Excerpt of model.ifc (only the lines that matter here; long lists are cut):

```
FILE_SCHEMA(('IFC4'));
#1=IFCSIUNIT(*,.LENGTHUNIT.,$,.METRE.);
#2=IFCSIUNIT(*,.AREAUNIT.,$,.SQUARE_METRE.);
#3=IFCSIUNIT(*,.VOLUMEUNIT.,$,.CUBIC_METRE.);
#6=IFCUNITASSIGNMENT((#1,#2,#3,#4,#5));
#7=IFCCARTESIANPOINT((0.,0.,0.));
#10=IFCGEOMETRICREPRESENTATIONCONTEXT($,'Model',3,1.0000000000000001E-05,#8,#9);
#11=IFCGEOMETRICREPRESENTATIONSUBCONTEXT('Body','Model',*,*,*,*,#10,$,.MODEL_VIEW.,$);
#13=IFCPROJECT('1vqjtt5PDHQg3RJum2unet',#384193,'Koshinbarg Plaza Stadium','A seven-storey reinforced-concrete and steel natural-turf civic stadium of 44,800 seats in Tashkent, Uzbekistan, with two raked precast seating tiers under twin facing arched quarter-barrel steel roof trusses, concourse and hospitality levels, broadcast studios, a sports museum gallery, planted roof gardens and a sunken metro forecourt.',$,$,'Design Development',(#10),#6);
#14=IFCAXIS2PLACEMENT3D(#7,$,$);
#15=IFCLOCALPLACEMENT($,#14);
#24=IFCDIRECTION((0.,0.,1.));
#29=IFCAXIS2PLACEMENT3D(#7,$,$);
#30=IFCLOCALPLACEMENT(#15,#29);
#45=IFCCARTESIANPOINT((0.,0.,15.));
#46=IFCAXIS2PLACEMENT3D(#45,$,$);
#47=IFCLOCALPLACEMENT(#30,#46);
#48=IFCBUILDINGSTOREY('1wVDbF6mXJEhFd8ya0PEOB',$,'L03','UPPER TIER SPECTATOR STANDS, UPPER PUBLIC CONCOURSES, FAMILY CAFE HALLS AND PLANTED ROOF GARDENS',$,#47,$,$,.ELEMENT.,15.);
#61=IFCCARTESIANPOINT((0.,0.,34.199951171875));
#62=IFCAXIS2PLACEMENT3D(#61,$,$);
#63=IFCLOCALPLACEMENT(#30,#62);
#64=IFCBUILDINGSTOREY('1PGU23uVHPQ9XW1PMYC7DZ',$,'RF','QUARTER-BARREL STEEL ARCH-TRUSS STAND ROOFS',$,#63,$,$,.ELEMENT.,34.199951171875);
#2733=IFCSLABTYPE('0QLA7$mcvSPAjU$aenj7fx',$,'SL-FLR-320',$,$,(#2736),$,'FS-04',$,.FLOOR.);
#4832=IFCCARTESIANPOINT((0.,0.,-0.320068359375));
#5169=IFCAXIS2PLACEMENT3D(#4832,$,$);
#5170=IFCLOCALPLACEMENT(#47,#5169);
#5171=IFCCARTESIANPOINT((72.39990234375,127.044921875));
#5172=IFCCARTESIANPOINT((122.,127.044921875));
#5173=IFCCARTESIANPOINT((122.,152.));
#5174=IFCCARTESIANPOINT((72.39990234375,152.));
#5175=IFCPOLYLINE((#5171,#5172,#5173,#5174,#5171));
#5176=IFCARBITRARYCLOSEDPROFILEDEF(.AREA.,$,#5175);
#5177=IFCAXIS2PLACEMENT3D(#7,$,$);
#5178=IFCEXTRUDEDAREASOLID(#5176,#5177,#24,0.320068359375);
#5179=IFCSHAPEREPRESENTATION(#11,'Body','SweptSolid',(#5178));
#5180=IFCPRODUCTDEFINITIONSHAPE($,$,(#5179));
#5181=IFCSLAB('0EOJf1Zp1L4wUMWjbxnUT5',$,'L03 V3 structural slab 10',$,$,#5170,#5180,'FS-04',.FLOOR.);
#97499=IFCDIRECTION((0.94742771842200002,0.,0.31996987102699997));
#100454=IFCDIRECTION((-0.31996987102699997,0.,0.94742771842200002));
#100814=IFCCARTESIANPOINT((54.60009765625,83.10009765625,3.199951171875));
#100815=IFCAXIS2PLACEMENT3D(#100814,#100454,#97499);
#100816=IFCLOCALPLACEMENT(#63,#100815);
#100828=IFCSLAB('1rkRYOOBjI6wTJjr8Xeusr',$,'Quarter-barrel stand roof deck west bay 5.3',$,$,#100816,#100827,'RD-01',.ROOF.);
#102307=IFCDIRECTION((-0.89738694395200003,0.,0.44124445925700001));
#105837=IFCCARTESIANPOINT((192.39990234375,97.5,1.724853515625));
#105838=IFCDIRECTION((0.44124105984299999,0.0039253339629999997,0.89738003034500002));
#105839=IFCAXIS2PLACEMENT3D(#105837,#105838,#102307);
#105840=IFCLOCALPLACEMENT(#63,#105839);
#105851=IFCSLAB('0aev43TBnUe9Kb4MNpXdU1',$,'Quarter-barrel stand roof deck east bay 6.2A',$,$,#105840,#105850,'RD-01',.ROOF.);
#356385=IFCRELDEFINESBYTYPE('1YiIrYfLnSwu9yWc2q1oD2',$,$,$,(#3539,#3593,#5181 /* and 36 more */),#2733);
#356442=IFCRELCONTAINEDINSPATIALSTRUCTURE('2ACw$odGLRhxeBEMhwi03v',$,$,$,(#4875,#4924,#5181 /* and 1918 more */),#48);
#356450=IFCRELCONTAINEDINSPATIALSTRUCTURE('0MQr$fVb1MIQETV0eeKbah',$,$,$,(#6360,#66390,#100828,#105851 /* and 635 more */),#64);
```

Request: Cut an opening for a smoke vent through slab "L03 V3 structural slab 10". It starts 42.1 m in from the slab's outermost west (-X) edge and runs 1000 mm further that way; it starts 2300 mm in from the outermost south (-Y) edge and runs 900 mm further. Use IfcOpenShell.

```python
import numpy as np
import ifcopenshell
import ifcopenshell.api.feature
import ifcopenshell.api.geometry
import ifcopenshell.api.root
import ifcopenshell.geom
import ifcopenshell.util.placement
import ifcopenshell.util.representation
import ifcopenshell.util.shape
import ifcopenshell.util.unit

model = ifcopenshell.open("model.ifc")
unit_scale = ifcopenshell.util.unit.calculate_unit_scale(model)
settings = ifcopenshell.geom.settings()


def volume(element):
    """Net volume in cubic metres, openings subtracted."""
    shape = ifcopenshell.geom.create_shape(settings, element)
    return ifcopenshell.util.shape.get_volume(shape.geometry)


slab = model.by_guid("0EOJf1Zp1L4wUMWjbxnUT5")
before = volume(slab)

# Extent in the slab's own axes, in metres. The edges named are its -X and -Y sides.
slab_shape = ifcopenshell.geom.create_shape(settings, slab)
vertices = ifcopenshell.util.shape.get_vertices(slab_shape.geometry)
x_min, y_min, bottom = vertices.min(axis=0)
top = vertices[:, 2].max()

opening = ifcopenshell.api.root.create_entity(model, ifc_class="IfcOpeningElement", name="Smoke vent opening", predefined_type="OPENING")
context = ifcopenshell.util.representation.get_context(model, "Model", "Body", "MODEL_VIEW")
width, depth = 1, 0.9
outline = [(0.0, 0.0), (width, 0.0), (width, depth), (0.0, depth), (0.0, 0.0)]
# Overshoot both faces by 50 mm so the cut is clean.
shape = ifcopenshell.api.geometry.add_slab_representation(
    model, context=context, depth=top - bottom + 0.1, polyline=outline
)
ifcopenshell.api.geometry.assign_representation(model, product=opening, representation=shape)

matrix = ifcopenshell.util.placement.get_local_placement(slab.ObjectPlacement)
matrix[:, 3] = matrix @ np.append(np.array([x_min + 42.1, y_min + 2.3, bottom - 0.05]) / unit_scale, 1.0)
ifcopenshell.api.geometry.edit_object_placement(model, product=opening, matrix=matrix, is_si=False)
ifcopenshell.api.feature.add_feature(model, feature=opening, element=slab)

after = volume(slab)

print(f"slab volume {before:.3f} -> {after:.3f} m3")

model.write("model-out.ifc")
```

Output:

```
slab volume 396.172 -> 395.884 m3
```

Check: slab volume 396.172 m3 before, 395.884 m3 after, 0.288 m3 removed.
